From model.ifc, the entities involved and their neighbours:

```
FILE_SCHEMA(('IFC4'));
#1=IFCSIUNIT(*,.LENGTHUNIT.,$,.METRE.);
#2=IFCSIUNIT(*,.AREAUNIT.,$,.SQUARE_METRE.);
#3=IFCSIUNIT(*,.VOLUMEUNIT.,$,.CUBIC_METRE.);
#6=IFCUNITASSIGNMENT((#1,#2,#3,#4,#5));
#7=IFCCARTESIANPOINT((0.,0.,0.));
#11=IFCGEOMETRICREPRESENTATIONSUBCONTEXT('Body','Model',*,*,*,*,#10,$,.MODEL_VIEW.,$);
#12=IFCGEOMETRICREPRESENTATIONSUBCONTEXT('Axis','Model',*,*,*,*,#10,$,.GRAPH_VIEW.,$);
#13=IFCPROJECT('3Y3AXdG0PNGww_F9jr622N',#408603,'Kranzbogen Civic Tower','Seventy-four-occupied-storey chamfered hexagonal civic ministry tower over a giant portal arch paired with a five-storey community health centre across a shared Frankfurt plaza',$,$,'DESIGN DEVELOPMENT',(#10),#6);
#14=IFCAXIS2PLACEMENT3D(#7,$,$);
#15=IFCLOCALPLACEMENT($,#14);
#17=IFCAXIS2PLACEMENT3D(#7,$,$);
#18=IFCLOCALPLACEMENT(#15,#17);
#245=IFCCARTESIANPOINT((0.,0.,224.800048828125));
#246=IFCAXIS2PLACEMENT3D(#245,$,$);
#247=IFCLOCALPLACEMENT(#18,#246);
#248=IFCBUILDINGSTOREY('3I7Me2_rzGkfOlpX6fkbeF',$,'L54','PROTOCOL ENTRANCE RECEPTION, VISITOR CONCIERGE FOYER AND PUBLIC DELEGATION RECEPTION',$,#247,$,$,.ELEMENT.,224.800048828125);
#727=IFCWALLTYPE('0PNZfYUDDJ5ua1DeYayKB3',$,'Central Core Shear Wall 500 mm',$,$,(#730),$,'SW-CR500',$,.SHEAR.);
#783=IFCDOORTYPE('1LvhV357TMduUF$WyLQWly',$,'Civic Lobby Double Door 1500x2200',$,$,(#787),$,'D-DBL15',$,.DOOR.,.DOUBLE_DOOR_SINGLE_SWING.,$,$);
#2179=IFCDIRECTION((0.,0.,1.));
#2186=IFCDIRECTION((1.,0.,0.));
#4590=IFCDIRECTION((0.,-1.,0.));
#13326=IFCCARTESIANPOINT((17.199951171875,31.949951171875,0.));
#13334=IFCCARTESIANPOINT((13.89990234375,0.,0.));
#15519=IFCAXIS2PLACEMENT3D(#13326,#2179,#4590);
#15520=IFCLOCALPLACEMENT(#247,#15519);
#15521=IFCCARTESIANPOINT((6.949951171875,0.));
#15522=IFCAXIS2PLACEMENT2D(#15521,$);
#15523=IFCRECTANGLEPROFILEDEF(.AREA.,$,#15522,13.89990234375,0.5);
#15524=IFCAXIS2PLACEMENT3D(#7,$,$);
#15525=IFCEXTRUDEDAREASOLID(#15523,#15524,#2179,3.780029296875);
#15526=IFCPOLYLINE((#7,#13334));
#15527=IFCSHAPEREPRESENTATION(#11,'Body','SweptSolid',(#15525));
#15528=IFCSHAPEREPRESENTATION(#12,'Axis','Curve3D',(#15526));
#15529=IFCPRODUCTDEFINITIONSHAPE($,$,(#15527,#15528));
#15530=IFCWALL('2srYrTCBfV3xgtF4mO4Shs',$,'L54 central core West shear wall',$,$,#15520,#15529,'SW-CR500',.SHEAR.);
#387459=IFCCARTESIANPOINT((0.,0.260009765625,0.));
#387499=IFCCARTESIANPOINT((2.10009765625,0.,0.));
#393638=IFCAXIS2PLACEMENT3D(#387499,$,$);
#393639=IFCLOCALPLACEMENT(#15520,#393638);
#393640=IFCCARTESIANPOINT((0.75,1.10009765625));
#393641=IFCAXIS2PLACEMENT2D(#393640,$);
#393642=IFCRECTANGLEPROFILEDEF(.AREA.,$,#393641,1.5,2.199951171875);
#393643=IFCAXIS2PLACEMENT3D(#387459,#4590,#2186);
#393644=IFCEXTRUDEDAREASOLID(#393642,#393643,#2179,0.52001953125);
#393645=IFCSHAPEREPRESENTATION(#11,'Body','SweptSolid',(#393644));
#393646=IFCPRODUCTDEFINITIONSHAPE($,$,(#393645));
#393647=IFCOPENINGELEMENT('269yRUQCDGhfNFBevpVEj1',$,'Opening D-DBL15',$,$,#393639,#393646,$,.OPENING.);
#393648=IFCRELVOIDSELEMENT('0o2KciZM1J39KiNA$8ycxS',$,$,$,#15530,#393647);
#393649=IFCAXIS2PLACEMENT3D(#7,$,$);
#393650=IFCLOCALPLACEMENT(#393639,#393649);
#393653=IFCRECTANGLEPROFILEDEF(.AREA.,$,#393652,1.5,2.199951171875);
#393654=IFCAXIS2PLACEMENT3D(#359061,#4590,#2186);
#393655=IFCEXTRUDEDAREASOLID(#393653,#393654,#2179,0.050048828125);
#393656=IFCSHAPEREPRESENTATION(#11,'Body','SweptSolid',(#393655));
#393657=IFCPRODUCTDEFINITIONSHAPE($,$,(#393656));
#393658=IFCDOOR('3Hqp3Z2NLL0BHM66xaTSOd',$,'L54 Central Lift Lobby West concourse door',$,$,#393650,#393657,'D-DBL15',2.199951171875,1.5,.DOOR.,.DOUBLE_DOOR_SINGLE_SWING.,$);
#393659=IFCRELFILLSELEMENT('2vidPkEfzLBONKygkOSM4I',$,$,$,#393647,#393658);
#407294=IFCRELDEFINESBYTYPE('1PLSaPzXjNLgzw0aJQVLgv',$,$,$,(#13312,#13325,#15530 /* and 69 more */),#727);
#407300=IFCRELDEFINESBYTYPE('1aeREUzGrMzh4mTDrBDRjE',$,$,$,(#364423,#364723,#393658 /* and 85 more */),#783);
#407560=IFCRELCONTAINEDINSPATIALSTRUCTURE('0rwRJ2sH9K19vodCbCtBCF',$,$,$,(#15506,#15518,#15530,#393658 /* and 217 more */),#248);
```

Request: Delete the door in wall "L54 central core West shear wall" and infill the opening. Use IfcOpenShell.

```python
import ifcopenshell
import ifcopenshell.api.feature
import ifcopenshell.api.root
import ifcopenshell.geom
import ifcopenshell.util.shape

model = ifcopenshell.open("model.ifc")
settings = ifcopenshell.geom.settings()


def volume(element):
    """Net volume in cubic metres, openings subtracted."""
    shape = ifcopenshell.geom.create_shape(settings, element)
    return ifcopenshell.util.shape.get_volume(shape.geometry)


door = model.by_guid("3Hqp3Z2NLL0BHM66xaTSOd")
opening = door.FillsVoids[0].RelatingOpeningElement
wall = opening.VoidsElements[0].RelatingBuildingElement
before = volume(wall)

ifcopenshell.api.root.remove_product(model, product=door)
ifcopenshell.api.feature.remove_feature(model, feature=opening)

after = volume(wall)

print(f"wall volume {before:.3f} -> {after:.3f} m3")

model.write("model_updated.ifc")
```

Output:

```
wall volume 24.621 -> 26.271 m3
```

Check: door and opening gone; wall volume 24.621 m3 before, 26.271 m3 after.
